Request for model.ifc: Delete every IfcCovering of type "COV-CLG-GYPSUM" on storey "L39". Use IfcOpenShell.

First a look at what the model holds.

```python
import ifcopenshell
import ifcopenshell.util.element

model = ifcopenshell.open("model.ifc")
print(model.schema)
storey = next(s for s in model.by_type("IfcBuildingStorey") if s.Name == "L39")
coverings = [e for e in ifcopenshell.util.element.get_decomposition(storey) if e.is_a("IfcCovering")]
seen = {}
for e in coverings:
    element_type = ifcopenshell.util.element.get_type(e)
    name = element_type.Name if element_type not in (None, e) else None
    seen[name] = seen.get(name, 0) + 1
for name, count in sorted(seen.items(), key=str):
    print(count, "x", name)
```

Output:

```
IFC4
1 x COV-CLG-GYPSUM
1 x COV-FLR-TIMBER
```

```python
import ifcopenshell
import ifcopenshell.api.root
import ifcopenshell.util.element

model = ifcopenshell.open("model.ifc")

storey = next(s for s in model.by_type("IfcBuildingStorey") if s.Name == "L39")
coverings = [e for e in ifcopenshell.util.element.get_decomposition(storey) if e.is_a("IfcCovering")]
targets = [e for e in coverings if (t := ifcopenshell.util.element.get_type(e)) not in (None, e) and t.Name == "COV-CLG-GYPSUM"]

for e in targets:
    ifcopenshell.api.root.remove_product(model, product=e)
print(len(targets), "removed")

model.write("model_edited.ifc")
```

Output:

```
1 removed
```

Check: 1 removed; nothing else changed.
